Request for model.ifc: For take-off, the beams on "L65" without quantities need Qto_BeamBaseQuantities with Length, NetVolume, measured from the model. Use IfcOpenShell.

First a look at what the model holds.

```python
import ifcopenshell
import ifcopenshell.util.element
import ifcopenshell.util.unit

model = ifcopenshell.open("model.ifc")
print(model.schema)
for unit_type in ("LENGTHUNIT", "AREAUNIT", "VOLUMEUNIT"):
    print(unit_type, ifcopenshell.util.unit.calculate_unit_scale(model, unit_type))
storey = next(s for s in model.by_type("IfcBuildingStorey") if s.Name == "L65")
beams = [e for e in ifcopenshell.util.element.get_decomposition(storey) if e.is_a("IfcBeam")]
for e in sorted(beams, key=lambda e: e.id()):
    print(e.id(), e.is_a(), e.Name, list(ifcopenshell.util.element.get_psets(e, qtos_only=True)), sep=" | ")
```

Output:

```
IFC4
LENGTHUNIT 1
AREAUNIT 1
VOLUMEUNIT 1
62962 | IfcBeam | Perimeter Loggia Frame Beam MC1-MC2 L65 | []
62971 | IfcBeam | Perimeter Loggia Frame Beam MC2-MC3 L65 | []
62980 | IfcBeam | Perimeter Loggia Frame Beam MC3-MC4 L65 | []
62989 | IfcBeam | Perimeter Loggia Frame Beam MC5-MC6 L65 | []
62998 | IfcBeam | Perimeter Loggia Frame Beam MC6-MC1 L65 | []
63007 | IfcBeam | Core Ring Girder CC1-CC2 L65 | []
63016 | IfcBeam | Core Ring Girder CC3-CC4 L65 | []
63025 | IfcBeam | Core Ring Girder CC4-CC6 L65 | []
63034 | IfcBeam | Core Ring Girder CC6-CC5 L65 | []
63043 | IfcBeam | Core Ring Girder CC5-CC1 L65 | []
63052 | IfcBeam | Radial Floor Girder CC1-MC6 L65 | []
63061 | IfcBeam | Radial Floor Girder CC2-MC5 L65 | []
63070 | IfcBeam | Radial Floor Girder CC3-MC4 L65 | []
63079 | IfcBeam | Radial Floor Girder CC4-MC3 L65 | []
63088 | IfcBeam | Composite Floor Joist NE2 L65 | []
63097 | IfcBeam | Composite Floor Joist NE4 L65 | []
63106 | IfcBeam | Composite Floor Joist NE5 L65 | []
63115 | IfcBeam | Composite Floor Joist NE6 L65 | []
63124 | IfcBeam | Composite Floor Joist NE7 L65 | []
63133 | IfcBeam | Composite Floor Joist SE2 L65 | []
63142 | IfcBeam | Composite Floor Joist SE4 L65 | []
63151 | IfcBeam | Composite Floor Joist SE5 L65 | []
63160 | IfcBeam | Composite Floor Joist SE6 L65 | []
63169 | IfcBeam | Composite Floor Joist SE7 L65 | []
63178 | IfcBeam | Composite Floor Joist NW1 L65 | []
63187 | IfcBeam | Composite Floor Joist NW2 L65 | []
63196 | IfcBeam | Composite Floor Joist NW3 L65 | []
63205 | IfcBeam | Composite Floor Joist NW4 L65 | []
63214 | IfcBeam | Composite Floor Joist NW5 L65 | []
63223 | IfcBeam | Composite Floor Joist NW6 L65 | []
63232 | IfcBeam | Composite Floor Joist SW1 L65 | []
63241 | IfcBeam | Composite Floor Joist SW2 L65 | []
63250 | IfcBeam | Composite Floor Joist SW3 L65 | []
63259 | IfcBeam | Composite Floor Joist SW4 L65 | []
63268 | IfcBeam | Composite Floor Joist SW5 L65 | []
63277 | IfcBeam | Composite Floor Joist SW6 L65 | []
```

```python
import ifcopenshell
import ifcopenshell.api.pset
import ifcopenshell.geom
import ifcopenshell.util.element
import ifcopenshell.util.shape
import ifcopenshell.util.unit

model = ifcopenshell.open("model.ifc")
unit_scale = ifcopenshell.util.unit.calculate_unit_scale(model)
volume_scale = ifcopenshell.util.unit.calculate_unit_scale(model, "VOLUMEUNIT")
settings = ifcopenshell.geom.settings()

storey = next(s for s in model.by_type("IfcBuildingStorey") if s.Name == "L65")
beams = [e for e in ifcopenshell.util.element.get_decomposition(storey) if e.is_a("IfcBeam")]

for e in sorted(beams, key=lambda e: e.id()):
    if ifcopenshell.util.element.get_psets(e, qtos_only=True, should_inherit=False):
        continue
    # Geometry comes back in metres, in the element's own axes.
    shape = ifcopenshell.geom.create_shape(settings, e)
    values = {
        "Length": ifcopenshell.util.shape.get_max_xyz(shape.geometry) / unit_scale,
        "NetVolume": ifcopenshell.util.shape.get_volume(shape.geometry) / volume_scale,
    }
    qto = ifcopenshell.api.pset.add_qto(model, product=e, name="Qto_BeamBaseQuantities")
    ifcopenshell.api.pset.edit_qto(model, qto=qto, properties=values)
    print(e.id(), {k: round(v, 3) for k, v in values.items()})

model.write("model_rev.ifc")
```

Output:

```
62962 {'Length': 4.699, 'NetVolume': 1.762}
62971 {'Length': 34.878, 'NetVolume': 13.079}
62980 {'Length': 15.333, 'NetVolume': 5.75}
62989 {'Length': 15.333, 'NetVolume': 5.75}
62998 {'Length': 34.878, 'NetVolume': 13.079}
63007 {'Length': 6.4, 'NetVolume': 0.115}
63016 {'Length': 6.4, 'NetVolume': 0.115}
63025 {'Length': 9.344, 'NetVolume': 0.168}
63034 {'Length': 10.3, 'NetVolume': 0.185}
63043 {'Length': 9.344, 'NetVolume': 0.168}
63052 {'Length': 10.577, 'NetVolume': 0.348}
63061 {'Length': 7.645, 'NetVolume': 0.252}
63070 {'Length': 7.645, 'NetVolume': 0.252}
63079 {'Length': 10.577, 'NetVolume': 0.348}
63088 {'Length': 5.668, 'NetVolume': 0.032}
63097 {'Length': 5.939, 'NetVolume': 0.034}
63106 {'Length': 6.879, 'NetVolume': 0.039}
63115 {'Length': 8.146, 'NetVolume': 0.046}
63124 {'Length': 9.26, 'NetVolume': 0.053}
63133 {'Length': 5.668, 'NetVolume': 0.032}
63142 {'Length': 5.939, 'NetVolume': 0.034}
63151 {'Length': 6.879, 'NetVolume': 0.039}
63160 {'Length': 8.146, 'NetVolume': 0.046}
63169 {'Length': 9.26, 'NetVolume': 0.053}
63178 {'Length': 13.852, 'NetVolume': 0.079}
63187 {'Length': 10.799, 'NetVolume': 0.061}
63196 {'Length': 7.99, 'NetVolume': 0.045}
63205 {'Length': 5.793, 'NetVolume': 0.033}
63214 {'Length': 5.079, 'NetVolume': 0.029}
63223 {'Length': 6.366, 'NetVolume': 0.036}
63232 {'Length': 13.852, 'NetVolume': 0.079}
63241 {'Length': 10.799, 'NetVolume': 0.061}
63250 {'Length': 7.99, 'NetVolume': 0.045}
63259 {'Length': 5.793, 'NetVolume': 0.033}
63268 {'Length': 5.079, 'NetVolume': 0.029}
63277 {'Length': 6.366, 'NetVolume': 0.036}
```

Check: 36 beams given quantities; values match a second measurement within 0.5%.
